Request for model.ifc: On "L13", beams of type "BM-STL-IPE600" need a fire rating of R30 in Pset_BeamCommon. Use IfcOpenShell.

First a look at what the model holds.

```python
import ifcopenshell
import ifcopenshell.util.element

model = ifcopenshell.open("model.ifc")
print(model.schema)
storey = next(s for s in model.by_type("IfcBuildingStorey") if s.Name == "L13")
beams = [e for e in ifcopenshell.util.element.get_decomposition(storey) if e.is_a("IfcBeam")]
seen = {}
for e in beams:
    element_type = ifcopenshell.util.element.get_type(e)
    key = (element_type.Name if element_type != e and element_type else None, ifcopenshell.util.element.get_pset(e, "Pset_BeamCommon", "FireRating"))
    seen[key] = seen.get(key, 0) + 1
for (name, value), count in sorted(seen.items(), key=str):
    print(count, "x", name, "|", value)
```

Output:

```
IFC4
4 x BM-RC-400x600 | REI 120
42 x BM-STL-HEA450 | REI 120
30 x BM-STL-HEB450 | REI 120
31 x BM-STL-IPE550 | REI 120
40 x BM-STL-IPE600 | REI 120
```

```python
import ifcopenshell
import ifcopenshell.api.pset
import ifcopenshell.util.element

model = ifcopenshell.open("model.ifc")

storey = next(s for s in model.by_type("IfcBuildingStorey") if s.Name == "L13")
beams = [e for e in ifcopenshell.util.element.get_decomposition(storey) if e.is_a("IfcBeam")]

count = 0
for e in beams:
    element_type = ifcopenshell.util.element.get_type(e)
    if element_type in (None, e) or element_type.Name != "BM-STL-IPE600":
        continue
    # add_pset returns the element's existing set when there is one.
    pset = ifcopenshell.api.pset.add_pset(model, product=e, name="Pset_BeamCommon")
    ifcopenshell.api.pset.edit_pset(model, pset=pset, properties={"FireRating": "R30"})
    count += 1

print(count, "beams updated")

model.write("model-out.ifc")
```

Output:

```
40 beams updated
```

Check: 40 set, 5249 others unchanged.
